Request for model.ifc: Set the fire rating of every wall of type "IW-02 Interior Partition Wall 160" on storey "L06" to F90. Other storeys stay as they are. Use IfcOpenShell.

First a look at what the model holds.

```python
import ifcopenshell
import ifcopenshell.util.element

model = ifcopenshell.open("model.ifc")
print(model.schema)
storey = next(s for s in model.by_type("IfcBuildingStorey") if s.Name == "L06")
walls = [e for e in ifcopenshell.util.element.get_decomposition(storey) if e.is_a("IfcWall")]
seen = {}
for e in walls:
    element_type = ifcopenshell.util.element.get_type(e)
    key = (element_type.Name if element_type != e and element_type else None, ifcopenshell.util.element.get_pset(e, "Pset_WallCommon", "FireRating"))
    seen[key] = seen.get(key, 0) + 1
for (name, value), count in sorted(seen.items(), key=str):
    print(count, "x", name, "|", value)
```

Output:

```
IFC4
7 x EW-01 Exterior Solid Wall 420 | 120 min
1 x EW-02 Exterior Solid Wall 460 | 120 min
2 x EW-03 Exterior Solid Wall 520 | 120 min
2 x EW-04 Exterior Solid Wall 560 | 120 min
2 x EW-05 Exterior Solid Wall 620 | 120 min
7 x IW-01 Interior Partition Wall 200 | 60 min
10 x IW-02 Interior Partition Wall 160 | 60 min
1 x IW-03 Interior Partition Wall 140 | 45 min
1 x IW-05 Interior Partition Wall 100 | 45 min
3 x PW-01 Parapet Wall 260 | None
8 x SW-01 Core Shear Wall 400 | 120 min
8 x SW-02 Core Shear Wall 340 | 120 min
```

```python
import ifcopenshell
import ifcopenshell.api.pset
import ifcopenshell.util.element

model = ifcopenshell.open("model.ifc")

storey = next(s for s in model.by_type("IfcBuildingStorey") if s.Name == "L06")
walls = [e for e in ifcopenshell.util.element.get_decomposition(storey) if e.is_a("IfcWall")]

count = 0
for e in walls:
    element_type = ifcopenshell.util.element.get_type(e)
    if element_type in (None, e) or element_type.Name != "IW-02 Interior Partition Wall 160":
        continue
    # add_pset returns the element's existing set when there is one.
    pset = ifcopenshell.api.pset.add_pset(model, product=e, name="Pset_WallCommon")
    ifcopenshell.api.pset.edit_pset(model, pset=pset, properties={"FireRating": "F90"})
    count += 1

print(count, "walls updated")

model.write("model_v2.ifc")
```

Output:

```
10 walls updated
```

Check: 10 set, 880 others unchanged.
